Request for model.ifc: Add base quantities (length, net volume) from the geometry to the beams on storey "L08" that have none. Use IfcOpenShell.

First a look at what the model holds.

```python
import ifcopenshell
import ifcopenshell.util.element
import ifcopenshell.util.unit

model = ifcopenshell.open("model.ifc")
print(model.schema)
for unit_type in ("LENGTHUNIT", "AREAUNIT", "VOLUMEUNIT"):
    print(unit_type, ifcopenshell.util.unit.calculate_unit_scale(model, unit_type))
storey = next(s for s in model.by_type("IfcBuildingStorey") if s.Name == "L08")
beams = [e for e in ifcopenshell.util.element.get_decomposition(storey) if e.is_a("IfcBeam")]
for e in sorted(beams, key=lambda e: e.id()):
    print(e.id(), e.is_a(), e.Name, list(ifcopenshell.util.element.get_psets(e, qtos_only=True)), sep=" | ")
```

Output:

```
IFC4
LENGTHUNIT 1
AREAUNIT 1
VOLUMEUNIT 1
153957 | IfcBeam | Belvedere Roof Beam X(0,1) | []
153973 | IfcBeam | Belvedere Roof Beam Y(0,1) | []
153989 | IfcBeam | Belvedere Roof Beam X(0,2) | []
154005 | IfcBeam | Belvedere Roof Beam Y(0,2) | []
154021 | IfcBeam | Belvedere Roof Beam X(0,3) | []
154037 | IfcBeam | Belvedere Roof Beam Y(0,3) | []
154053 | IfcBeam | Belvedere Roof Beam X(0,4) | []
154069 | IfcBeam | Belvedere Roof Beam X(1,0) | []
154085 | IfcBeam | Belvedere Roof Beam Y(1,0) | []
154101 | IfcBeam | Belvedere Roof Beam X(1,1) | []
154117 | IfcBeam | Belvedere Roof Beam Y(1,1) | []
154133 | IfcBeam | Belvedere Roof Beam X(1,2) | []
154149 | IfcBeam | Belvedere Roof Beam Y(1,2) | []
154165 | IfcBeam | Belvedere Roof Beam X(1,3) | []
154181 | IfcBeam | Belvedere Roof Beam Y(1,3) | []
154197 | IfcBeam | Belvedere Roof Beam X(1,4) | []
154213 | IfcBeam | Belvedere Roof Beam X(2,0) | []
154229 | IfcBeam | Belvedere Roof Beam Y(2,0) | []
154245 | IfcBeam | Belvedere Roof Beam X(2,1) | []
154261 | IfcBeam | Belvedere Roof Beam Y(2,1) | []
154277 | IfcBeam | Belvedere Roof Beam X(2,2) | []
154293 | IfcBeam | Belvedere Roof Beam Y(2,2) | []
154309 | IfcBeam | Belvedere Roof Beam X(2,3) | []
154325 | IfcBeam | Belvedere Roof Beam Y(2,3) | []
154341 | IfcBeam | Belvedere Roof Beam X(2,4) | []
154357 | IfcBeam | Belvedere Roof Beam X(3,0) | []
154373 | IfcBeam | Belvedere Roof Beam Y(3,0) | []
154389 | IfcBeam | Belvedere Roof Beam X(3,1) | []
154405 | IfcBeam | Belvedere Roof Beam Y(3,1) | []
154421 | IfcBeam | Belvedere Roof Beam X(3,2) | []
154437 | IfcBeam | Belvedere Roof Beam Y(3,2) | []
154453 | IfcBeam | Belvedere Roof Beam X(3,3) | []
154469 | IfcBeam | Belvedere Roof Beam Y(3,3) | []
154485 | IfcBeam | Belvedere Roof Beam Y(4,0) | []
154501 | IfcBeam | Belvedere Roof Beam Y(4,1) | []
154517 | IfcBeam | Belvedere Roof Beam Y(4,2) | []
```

```python
import ifcopenshell
import ifcopenshell.api.pset
import ifcopenshell.geom
import ifcopenshell.util.element
import ifcopenshell.util.shape
import ifcopenshell.util.unit

model = ifcopenshell.open("model.ifc")
unit_scale = ifcopenshell.util.unit.calculate_unit_scale(model)
volume_scale = ifcopenshell.util.unit.calculate_unit_scale(model, "VOLUMEUNIT")
settings = ifcopenshell.geom.settings()

storey = next(s for s in model.by_type("IfcBuildingStorey") if s.Name == "L08")
beams = [e for e in ifcopenshell.util.element.get_decomposition(storey) if e.is_a("IfcBeam")]

for e in sorted(beams, key=lambda e: e.id()):
    if ifcopenshell.util.element.get_psets(e, qtos_only=True, should_inherit=False):
        continue
    # Geometry comes back in metres, in the element's own axes.
    shape = ifcopenshell.geom.create_shape(settings, e)
    values = {
        "Length": ifcopenshell.util.shape.get_max_xyz(shape.geometry) / unit_scale,
        "NetVolume": ifcopenshell.util.shape.get_volume(shape.geometry) / volume_scale,
    }
    qto = ifcopenshell.api.pset.add_qto(model, product=e, name="Qto_BeamBaseQuantities")
    ifcopenshell.api.pset.edit_qto(model, qto=qto, properties=values)
    print(e.id(), {k: round(v, 3) for k, v in values.items()})

model.write("model_updated.ifc")
```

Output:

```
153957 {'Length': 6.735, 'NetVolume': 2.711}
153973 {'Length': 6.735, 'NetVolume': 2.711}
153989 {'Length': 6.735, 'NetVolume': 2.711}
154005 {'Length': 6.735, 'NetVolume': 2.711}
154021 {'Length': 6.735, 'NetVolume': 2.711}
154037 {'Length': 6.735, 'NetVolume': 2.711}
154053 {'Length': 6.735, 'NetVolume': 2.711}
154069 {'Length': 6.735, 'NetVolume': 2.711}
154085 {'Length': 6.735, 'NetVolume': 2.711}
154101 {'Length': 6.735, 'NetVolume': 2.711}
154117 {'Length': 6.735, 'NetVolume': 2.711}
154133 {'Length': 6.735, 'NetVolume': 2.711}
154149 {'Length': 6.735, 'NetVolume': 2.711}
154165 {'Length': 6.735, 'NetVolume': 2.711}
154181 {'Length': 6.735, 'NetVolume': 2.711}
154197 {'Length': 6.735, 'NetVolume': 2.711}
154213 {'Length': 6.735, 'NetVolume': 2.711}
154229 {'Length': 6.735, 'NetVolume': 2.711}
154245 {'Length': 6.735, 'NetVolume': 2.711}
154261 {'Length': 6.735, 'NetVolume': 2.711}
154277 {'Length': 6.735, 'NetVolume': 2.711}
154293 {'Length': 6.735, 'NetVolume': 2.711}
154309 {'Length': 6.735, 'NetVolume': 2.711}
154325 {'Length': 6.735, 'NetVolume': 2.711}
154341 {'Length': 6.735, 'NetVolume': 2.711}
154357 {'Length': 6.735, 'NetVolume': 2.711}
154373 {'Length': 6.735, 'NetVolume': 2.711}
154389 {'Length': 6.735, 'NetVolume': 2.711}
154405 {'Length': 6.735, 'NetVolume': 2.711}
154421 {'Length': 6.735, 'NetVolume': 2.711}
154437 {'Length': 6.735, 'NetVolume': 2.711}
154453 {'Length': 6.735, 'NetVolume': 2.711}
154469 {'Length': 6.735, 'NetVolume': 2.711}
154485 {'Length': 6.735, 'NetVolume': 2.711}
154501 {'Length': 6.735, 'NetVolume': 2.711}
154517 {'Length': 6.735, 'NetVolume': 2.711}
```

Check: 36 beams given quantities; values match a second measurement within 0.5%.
